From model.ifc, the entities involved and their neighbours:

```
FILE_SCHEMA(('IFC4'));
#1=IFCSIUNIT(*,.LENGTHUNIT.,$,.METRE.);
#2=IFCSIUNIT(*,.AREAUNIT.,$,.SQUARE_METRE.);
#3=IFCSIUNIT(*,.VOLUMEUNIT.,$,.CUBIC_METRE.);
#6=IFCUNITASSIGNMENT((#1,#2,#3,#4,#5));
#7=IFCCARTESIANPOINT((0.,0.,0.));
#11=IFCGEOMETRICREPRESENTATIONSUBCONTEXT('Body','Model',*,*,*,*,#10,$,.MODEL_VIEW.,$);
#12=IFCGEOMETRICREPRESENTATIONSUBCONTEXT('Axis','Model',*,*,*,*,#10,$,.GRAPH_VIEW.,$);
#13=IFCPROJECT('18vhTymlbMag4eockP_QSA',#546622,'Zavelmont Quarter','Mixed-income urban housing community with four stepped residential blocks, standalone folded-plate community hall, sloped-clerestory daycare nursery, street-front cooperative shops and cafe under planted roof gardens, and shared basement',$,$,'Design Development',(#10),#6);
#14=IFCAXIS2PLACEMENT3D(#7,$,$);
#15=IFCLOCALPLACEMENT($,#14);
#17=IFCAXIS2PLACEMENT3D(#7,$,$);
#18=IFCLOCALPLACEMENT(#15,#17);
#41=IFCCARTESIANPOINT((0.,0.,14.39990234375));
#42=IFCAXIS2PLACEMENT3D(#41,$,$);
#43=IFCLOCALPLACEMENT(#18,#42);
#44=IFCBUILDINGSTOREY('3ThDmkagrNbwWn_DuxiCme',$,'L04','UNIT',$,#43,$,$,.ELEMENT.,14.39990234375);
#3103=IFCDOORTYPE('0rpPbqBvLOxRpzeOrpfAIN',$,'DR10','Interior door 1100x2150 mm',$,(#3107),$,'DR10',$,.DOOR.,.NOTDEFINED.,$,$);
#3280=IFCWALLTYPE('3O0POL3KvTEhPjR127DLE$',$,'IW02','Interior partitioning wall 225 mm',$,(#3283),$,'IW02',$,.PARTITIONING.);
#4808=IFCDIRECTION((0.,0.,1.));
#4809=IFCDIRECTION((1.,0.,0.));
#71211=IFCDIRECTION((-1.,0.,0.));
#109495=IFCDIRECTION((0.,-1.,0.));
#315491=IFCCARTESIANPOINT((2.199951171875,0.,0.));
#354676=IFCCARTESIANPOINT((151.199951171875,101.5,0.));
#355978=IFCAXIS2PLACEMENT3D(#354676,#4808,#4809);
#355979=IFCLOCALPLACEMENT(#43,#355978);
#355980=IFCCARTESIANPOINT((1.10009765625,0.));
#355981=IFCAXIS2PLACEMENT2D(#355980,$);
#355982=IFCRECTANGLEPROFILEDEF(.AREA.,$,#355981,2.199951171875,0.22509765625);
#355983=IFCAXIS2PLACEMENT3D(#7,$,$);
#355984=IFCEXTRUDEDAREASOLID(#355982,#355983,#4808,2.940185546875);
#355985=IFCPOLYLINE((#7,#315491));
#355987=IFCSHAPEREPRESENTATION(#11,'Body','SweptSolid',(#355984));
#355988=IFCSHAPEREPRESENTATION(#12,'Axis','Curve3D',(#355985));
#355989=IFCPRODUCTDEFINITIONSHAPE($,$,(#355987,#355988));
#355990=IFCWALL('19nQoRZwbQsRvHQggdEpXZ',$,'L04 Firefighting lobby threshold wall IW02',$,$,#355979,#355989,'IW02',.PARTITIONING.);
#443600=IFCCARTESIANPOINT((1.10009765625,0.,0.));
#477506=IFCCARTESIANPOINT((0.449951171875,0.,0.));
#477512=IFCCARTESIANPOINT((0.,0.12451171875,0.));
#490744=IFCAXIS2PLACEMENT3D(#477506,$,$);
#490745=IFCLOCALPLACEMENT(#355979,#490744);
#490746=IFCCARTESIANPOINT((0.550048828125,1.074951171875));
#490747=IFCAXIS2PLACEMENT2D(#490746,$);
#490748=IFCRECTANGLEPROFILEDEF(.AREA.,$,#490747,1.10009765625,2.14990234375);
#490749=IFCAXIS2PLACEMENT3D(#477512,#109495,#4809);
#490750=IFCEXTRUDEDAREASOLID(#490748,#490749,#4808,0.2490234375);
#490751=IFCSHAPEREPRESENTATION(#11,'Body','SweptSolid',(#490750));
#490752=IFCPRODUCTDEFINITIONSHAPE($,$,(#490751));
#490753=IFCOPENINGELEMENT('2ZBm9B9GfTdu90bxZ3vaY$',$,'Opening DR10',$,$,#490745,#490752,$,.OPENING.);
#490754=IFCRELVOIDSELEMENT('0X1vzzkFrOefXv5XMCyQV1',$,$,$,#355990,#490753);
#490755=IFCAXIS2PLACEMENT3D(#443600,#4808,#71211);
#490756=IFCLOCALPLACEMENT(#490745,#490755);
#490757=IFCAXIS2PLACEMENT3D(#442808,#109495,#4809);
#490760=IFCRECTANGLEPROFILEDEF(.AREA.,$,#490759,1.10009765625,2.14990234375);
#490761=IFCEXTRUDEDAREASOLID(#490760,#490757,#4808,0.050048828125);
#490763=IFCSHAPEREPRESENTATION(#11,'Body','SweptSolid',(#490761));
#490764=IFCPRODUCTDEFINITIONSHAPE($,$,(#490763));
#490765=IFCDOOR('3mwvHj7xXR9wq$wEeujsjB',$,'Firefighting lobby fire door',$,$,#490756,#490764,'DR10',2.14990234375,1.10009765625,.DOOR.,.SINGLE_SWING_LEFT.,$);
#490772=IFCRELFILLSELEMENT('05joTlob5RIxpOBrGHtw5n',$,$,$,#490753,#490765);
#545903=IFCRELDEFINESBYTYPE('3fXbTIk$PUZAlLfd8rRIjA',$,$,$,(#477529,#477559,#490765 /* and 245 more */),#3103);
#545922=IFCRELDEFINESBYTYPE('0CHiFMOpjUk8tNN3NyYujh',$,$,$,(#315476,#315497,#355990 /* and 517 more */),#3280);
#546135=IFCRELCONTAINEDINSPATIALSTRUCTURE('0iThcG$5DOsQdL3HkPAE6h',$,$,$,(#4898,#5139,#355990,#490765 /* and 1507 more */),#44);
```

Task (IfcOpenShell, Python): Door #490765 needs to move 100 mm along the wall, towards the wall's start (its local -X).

```python
import ifcopenshell
import ifcopenshell.api.geometry
import ifcopenshell.util.placement
import ifcopenshell.util.unit

model = ifcopenshell.open("model.ifc")
unit_scale = ifcopenshell.util.unit.calculate_unit_scale(model)

door = model.by_id(490765)
opening = door.FillsVoids[0].RelatingOpeningElement
wall = opening.VoidsElements[0].RelatingBuildingElement

wall_matrix = ifcopenshell.util.placement.get_local_placement(wall.ObjectPlacement)
shift = wall_matrix[:3, 0] * -0.1 / unit_scale
before = ifcopenshell.util.placement.get_local_placement(door.ObjectPlacement)[:3, 3].copy()

# The door is placed relative to its opening, so it follows when the opening moves.
matrix = ifcopenshell.util.placement.get_local_placement(opening.ObjectPlacement)
matrix[:3, 3] += shift
ifcopenshell.api.geometry.edit_object_placement(
    model, product=opening, matrix=matrix, is_si=False, should_transform_children=True
)

after = ifcopenshell.util.placement.get_local_placement(door.ObjectPlacement)[:3, 3]
print("door moved by", (after - before).round(3) + 0.0)

model.write("model_updated.ifc")
```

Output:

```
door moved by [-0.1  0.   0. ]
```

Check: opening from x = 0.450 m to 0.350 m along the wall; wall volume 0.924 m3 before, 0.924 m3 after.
